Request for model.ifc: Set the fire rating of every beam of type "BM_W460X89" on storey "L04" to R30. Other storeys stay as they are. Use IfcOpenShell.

First a look at what the model holds.

```python
import ifcopenshell
import ifcopenshell.util.element

model = ifcopenshell.open("model.ifc")
print(model.schema)
storey = next(s for s in model.by_type("IfcBuildingStorey") if s.Name == "L04")
beams = [e for e in ifcopenshell.util.element.get_decomposition(storey) if e.is_a("IfcBeam")]
seen = {}
for e in beams:
    element_type = ifcopenshell.util.element.get_type(e)
    key = (element_type.Name if element_type != e and element_type else None, ifcopenshell.util.element.get_pset(e, "Pset_BeamCommon", "FireRating"))
    seen[key] = seen.get(key, 0) + 1
for (name, value), count in sorted(seen.items(), key=str):
    print(count, "x", name, "|", value)
```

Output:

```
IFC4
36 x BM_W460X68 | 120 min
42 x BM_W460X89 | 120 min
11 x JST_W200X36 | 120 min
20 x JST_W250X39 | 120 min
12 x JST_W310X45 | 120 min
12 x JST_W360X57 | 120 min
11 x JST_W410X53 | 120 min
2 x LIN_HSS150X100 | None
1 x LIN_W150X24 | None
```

```python
import ifcopenshell
import ifcopenshell.api.pset
import ifcopenshell.util.element

model = ifcopenshell.open("model.ifc")

storey = next(s for s in model.by_type("IfcBuildingStorey") if s.Name == "L04")
beams = [e for e in ifcopenshell.util.element.get_decomposition(storey) if e.is_a("IfcBeam")]

count = 0
for e in beams:
    element_type = ifcopenshell.util.element.get_type(e)
    if element_type in (None, e) or element_type.Name != "BM_W460X89":
        continue
    # add_pset returns the element's existing set when there is one.
    pset = ifcopenshell.api.pset.add_pset(model, product=e, name="Pset_BeamCommon")
    ifcopenshell.api.pset.edit_pset(model, pset=pset, properties={"FireRating": "R30"})
    count += 1

print(count, "beams updated")

model.write("model-out.ifc")
```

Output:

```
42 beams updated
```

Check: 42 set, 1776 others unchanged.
